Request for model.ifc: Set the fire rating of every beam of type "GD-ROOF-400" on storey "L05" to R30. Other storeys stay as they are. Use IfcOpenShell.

First a look at what the model holds.

```python
import ifcopenshell
import ifcopenshell.util.element

model = ifcopenshell.open("model.ifc")
print(model.schema)
storey = next(s for s in model.by_type("IfcBuildingStorey") if s.Name == "L05")
beams = [e for e in ifcopenshell.util.element.get_decomposition(storey) if e.is_a("IfcBeam")]
seen = {}
for e in beams:
    element_type = ifcopenshell.util.element.get_type(e)
    key = (element_type.Name if element_type != e and element_type else None, ifcopenshell.util.element.get_pset(e, "Pset_BeamCommon", "FireRating"))
    seen[key] = seen.get(key, 0) + 1
for (name, value), count in sorted(seen.items(), key=str):
    print(count, "x", name, "|", value)
```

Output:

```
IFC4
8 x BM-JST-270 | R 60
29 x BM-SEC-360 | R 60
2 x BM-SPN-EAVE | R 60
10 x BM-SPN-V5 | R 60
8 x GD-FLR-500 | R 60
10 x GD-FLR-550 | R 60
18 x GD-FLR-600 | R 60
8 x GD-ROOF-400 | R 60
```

```python
import ifcopenshell
import ifcopenshell.api.pset
import ifcopenshell.util.element

model = ifcopenshell.open("model.ifc")

storey = next(s for s in model.by_type("IfcBuildingStorey") if s.Name == "L05")
beams = [e for e in ifcopenshell.util.element.get_decomposition(storey) if e.is_a("IfcBeam")]

count = 0
for e in beams:
    element_type = ifcopenshell.util.element.get_type(e)
    if element_type in (None, e) or element_type.Name != "GD-ROOF-400":
        continue
    # add_pset returns the element's existing set when there is one.
    pset = ifcopenshell.api.pset.add_pset(model, product=e, name="Pset_BeamCommon")
    ifcopenshell.api.pset.edit_pset(model, pset=pset, properties={"FireRating": "R30"})
    count += 1

print(count, "beams updated")

model.write("model_updated.ifc")
```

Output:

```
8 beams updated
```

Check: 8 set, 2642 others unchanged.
